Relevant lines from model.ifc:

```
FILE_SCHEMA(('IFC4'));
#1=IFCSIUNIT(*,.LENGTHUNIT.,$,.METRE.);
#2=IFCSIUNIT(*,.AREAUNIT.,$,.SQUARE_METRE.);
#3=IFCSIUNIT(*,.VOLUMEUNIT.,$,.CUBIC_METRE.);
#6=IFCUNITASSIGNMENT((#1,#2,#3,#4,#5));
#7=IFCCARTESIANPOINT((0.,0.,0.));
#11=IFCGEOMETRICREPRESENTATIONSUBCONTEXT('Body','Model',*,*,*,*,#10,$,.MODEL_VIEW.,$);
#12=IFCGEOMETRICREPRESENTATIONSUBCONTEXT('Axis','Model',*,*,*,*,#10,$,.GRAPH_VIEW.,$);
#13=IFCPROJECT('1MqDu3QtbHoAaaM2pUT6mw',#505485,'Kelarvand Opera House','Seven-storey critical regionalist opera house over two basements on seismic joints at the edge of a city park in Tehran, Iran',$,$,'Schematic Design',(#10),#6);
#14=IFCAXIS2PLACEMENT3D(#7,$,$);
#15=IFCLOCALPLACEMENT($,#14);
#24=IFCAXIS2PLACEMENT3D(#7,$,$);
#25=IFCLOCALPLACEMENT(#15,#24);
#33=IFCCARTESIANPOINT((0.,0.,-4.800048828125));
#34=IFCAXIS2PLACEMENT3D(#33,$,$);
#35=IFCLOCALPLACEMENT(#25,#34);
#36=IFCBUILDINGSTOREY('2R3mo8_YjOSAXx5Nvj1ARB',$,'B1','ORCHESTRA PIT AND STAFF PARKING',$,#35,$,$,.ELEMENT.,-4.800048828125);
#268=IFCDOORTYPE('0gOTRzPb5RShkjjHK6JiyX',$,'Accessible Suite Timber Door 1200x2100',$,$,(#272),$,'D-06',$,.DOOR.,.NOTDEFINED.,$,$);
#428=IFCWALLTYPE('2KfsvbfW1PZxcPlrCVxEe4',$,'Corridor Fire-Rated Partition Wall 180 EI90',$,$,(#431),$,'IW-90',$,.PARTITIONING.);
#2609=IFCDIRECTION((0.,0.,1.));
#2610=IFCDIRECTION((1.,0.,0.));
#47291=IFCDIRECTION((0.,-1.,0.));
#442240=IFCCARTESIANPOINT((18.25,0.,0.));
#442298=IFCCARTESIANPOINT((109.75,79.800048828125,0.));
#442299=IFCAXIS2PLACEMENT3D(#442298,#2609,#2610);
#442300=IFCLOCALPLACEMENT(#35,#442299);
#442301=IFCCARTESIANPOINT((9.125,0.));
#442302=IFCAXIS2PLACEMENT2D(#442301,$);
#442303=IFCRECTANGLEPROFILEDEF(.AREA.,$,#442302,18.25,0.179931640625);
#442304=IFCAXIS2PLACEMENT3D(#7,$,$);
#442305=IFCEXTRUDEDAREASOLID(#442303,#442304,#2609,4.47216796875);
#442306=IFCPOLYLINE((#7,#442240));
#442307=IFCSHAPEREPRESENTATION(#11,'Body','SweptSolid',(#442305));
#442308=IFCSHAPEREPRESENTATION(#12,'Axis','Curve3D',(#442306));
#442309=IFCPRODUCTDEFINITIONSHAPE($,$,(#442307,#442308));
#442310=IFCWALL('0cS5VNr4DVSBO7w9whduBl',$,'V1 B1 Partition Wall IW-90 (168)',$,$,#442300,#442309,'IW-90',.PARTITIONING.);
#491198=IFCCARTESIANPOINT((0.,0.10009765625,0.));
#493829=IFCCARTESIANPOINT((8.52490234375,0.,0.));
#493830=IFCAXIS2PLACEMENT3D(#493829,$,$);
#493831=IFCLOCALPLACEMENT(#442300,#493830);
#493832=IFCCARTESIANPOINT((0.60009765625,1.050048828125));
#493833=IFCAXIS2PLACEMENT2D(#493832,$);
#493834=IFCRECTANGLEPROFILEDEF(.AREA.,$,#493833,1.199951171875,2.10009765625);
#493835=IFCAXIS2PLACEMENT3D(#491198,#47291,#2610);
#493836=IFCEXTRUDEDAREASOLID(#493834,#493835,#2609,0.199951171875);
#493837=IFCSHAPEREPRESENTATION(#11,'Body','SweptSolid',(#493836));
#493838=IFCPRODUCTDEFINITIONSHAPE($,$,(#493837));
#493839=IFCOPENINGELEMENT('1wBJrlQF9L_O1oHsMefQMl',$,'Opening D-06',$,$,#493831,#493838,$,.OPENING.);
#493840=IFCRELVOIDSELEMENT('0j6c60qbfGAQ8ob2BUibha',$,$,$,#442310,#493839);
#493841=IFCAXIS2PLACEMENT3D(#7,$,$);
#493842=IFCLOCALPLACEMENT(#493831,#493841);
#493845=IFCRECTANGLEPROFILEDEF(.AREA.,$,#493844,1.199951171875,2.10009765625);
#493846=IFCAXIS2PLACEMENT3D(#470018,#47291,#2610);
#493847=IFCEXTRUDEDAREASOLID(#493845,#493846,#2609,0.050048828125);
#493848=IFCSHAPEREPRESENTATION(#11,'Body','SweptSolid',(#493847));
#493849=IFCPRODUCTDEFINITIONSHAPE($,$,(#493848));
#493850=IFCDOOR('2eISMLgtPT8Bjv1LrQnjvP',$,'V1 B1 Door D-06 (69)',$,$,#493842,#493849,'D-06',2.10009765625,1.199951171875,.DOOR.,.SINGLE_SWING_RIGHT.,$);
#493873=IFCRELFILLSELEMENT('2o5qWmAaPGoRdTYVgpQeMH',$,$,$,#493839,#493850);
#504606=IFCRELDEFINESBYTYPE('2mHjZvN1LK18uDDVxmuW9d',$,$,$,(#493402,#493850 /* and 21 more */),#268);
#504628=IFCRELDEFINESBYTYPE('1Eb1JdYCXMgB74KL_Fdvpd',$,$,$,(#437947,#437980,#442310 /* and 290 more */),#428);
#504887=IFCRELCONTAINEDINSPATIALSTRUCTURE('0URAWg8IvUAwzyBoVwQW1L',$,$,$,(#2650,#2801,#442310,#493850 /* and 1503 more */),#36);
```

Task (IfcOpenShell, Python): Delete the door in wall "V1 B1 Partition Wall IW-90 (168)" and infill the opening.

```python
import ifcopenshell
import ifcopenshell.api.feature
import ifcopenshell.api.root
import ifcopenshell.geom
import ifcopenshell.util.shape

model = ifcopenshell.open("model.ifc")
settings = ifcopenshell.geom.settings()


def volume(element):
    """Net volume in cubic metres, openings subtracted."""
    shape = ifcopenshell.geom.create_shape(settings, element)
    return ifcopenshell.util.shape.get_volume(shape.geometry)


door = model.by_guid("2eISMLgtPT8Bjv1LrQnjvP")
opening = door.FillsVoids[0].RelatingOpeningElement
wall = opening.VoidsElements[0].RelatingBuildingElement
before = volume(wall)

ifcopenshell.api.root.remove_product(model, product=door)
ifcopenshell.api.feature.remove_feature(model, feature=opening)

after = volume(wall)

print(f"wall volume {before:.3f} -> {after:.3f} m3")

model.write("model-out.ifc")
```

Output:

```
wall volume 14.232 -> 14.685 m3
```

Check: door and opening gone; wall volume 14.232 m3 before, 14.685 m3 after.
